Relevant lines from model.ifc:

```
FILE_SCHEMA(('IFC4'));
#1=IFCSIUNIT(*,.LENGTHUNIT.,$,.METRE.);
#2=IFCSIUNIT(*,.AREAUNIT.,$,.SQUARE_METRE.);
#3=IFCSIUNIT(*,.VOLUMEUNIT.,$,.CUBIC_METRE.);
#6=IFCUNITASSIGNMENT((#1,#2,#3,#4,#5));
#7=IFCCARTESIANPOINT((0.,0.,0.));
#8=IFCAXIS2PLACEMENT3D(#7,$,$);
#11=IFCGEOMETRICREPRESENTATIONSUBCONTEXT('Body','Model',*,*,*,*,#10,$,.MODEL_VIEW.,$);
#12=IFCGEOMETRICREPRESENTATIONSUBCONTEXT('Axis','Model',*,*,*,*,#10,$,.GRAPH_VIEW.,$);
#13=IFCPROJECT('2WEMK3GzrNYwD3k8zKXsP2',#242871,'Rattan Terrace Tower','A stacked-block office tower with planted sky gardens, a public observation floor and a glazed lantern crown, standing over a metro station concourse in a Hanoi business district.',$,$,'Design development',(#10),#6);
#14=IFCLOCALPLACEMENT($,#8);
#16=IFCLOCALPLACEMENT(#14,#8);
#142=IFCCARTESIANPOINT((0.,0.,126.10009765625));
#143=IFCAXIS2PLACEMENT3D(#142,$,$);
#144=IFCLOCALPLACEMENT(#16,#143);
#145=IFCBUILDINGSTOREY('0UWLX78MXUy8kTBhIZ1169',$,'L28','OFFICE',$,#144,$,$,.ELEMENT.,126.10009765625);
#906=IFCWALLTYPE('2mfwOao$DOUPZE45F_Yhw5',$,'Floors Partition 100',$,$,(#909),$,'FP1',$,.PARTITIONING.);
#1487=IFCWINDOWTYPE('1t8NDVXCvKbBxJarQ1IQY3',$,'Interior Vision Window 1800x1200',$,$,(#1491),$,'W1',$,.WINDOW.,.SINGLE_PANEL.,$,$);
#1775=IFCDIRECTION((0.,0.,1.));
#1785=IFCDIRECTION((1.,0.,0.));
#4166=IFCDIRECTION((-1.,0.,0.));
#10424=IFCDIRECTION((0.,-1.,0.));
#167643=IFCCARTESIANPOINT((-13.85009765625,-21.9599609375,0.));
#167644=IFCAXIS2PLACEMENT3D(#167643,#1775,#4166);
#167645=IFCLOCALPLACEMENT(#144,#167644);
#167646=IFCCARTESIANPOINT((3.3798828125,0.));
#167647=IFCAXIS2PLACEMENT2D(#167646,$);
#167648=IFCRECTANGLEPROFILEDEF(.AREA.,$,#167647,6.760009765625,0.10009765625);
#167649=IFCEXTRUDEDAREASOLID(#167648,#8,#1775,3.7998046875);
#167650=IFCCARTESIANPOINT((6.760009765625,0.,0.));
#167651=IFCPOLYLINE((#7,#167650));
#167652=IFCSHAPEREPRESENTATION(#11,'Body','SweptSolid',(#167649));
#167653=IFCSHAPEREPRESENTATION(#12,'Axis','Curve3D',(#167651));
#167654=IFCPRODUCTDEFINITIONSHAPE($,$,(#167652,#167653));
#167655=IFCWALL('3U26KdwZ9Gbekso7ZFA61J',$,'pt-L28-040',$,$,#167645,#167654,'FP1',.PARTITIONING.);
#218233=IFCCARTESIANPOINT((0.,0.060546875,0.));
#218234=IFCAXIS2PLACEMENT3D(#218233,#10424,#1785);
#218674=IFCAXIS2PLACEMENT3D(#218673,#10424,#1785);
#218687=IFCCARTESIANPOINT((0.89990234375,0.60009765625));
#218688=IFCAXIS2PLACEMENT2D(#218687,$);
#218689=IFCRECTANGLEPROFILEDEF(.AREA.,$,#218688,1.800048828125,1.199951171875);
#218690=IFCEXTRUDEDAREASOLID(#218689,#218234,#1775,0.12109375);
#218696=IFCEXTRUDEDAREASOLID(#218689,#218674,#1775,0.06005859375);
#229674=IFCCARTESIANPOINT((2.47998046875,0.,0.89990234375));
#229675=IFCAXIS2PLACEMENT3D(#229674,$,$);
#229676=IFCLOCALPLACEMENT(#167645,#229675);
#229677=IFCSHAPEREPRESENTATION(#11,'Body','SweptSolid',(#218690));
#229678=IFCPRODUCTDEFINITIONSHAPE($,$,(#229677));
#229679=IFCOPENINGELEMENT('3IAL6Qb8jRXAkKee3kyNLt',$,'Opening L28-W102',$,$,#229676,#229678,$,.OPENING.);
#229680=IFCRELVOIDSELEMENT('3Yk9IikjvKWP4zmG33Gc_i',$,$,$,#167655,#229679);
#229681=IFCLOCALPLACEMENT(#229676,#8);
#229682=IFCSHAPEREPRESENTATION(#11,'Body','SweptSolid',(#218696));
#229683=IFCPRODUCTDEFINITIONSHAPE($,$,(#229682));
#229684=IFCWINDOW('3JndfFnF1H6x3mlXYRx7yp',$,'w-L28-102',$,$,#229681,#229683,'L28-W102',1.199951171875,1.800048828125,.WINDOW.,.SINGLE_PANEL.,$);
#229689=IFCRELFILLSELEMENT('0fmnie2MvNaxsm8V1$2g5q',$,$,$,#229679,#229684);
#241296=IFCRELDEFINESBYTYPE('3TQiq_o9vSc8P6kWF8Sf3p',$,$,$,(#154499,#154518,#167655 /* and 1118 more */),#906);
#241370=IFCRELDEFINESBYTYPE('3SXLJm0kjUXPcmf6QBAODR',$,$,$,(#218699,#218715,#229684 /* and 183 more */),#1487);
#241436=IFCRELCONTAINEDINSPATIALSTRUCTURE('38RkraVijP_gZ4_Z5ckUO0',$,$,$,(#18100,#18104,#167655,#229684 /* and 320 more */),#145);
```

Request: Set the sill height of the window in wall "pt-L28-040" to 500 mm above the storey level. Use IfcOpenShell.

```python
import numpy as np
import ifcopenshell
import ifcopenshell.api.geometry
import ifcopenshell.geom
import ifcopenshell.util.element
import ifcopenshell.util.placement
import ifcopenshell.util.shape
import ifcopenshell.util.unit

model = ifcopenshell.open("model.ifc")
unit_scale = ifcopenshell.util.unit.calculate_unit_scale(model)

window = model.by_guid("3JndfFnF1H6x3mlXYRx7yp")
opening = window.FillsVoids[0].RelatingOpeningElement
storey = ifcopenshell.util.element.get_container(window, ifc_class="IfcBuildingStorey")
level = ifcopenshell.util.placement.get_local_placement(storey.ObjectPlacement)[2, 3]

# The opening's origin need not be at the sill, so measure its lowest point.
shape = ifcopenshell.geom.create_shape(ifcopenshell.geom.settings(), opening)
bottom = ifcopenshell.util.shape.get_shape_bottom_elevation(shape, shape.geometry) / unit_scale
dz = level + 0.5 - bottom

shift = np.array([0.0, 0.0, dz])
# The window is placed relative to its opening, so it follows when the opening moves.
matrix = ifcopenshell.util.placement.get_local_placement(opening.ObjectPlacement)
matrix[:3, 3] += shift
ifcopenshell.api.geometry.edit_object_placement(
    model, product=opening, matrix=matrix, is_si=False, should_transform_children=True
)

print(f"moved by {dz * unit_scale:+.3f} m")

model.write("model_rev.ifc")
```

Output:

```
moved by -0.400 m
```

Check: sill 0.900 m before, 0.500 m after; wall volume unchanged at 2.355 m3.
